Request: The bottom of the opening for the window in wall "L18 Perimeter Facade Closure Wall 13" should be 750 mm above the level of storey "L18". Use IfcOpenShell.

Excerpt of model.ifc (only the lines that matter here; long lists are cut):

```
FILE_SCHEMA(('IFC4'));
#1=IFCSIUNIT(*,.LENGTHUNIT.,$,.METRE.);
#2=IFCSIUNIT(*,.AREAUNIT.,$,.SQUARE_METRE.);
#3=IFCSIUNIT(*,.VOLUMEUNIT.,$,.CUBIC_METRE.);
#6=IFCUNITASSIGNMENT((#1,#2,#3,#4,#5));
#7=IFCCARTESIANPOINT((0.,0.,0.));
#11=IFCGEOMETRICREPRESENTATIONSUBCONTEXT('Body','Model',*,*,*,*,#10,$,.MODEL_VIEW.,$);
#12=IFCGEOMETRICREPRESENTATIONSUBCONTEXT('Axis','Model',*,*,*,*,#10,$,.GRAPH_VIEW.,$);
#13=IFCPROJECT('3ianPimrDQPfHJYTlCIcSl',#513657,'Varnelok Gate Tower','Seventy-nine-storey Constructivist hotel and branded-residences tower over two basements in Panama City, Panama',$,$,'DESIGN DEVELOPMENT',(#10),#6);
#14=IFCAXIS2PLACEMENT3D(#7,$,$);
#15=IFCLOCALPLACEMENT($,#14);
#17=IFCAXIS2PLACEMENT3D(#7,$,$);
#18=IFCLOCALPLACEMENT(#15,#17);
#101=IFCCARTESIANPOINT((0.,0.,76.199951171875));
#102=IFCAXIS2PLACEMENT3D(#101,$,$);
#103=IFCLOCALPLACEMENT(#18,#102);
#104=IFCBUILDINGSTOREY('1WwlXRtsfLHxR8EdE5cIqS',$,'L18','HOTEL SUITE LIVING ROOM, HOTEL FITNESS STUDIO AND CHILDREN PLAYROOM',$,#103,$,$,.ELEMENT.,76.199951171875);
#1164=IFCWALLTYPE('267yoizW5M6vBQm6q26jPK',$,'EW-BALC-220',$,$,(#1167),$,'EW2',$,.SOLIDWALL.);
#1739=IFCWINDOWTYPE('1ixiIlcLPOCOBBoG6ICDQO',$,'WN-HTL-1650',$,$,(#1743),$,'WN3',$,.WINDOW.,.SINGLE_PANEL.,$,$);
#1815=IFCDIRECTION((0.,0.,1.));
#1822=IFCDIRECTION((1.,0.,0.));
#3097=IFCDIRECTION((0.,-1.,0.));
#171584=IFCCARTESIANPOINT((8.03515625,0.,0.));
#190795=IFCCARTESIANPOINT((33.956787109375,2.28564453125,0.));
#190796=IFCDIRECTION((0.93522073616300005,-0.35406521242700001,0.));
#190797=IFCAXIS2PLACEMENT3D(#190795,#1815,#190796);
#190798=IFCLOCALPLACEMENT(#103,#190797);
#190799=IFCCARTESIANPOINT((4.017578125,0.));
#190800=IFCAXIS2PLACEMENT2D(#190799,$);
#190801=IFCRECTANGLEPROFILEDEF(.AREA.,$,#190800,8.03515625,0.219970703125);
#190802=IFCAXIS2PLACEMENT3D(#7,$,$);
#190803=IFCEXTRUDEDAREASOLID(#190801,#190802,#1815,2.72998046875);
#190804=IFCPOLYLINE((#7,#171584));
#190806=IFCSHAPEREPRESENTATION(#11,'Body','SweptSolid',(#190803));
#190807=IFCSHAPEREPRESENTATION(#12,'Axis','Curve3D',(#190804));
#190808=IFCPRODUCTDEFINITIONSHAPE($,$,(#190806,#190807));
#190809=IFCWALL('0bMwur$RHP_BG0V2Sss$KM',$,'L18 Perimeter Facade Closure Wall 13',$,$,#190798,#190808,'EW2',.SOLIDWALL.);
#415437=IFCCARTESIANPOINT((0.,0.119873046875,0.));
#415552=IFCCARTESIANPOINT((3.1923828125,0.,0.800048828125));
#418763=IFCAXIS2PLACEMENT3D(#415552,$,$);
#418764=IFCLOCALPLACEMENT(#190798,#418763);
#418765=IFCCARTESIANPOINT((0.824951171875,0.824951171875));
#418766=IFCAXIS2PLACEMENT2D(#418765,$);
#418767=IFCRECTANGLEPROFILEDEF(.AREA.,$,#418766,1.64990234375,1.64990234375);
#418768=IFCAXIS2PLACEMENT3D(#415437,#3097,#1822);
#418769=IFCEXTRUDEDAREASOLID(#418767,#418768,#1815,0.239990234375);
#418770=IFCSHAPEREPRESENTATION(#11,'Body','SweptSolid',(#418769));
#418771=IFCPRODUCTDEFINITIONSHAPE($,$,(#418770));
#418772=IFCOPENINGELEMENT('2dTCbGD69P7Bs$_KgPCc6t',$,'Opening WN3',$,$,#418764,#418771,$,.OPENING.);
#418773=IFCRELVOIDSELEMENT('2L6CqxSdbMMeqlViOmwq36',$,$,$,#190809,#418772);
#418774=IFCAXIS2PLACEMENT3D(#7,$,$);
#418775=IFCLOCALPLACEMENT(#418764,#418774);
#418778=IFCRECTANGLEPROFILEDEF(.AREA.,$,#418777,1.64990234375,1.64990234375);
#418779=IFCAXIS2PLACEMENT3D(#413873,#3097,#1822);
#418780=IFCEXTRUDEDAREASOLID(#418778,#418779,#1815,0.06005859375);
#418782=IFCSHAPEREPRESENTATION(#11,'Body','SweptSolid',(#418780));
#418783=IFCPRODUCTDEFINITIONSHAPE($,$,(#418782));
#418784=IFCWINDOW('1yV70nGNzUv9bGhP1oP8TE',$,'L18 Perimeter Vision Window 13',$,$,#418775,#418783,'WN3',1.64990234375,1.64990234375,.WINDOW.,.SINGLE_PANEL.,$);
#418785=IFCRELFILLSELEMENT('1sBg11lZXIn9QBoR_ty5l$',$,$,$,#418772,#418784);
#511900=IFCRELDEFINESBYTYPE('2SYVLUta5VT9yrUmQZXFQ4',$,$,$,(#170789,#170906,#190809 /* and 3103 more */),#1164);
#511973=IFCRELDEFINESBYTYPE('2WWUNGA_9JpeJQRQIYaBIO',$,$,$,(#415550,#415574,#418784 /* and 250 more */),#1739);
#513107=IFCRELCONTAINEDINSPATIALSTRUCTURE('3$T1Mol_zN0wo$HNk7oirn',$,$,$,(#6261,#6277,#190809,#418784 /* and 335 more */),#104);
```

```python
import numpy as np
import ifcopenshell
import ifcopenshell.api.geometry
import ifcopenshell.geom
import ifcopenshell.util.element
import ifcopenshell.util.placement
import ifcopenshell.util.shape
import ifcopenshell.util.unit

model = ifcopenshell.open("model.ifc")
unit_scale = ifcopenshell.util.unit.calculate_unit_scale(model)

window = model.by_guid("1yV70nGNzUv9bGhP1oP8TE")
opening = window.FillsVoids[0].RelatingOpeningElement
storey = ifcopenshell.util.element.get_container(window, ifc_class="IfcBuildingStorey")
level = ifcopenshell.util.placement.get_local_placement(storey.ObjectPlacement)[2, 3]

# The opening's origin need not be at the sill, so measure its lowest point.
shape = ifcopenshell.geom.create_shape(ifcopenshell.geom.settings(), opening)
bottom = ifcopenshell.util.shape.get_shape_bottom_elevation(shape, shape.geometry) / unit_scale
dz = level + 0.75 - bottom

shift = np.array([0.0, 0.0, dz])
# The window is placed relative to its opening, so it follows when the opening moves.
matrix = ifcopenshell.util.placement.get_local_placement(opening.ObjectPlacement)
matrix[:3, 3] += shift
ifcopenshell.api.geometry.edit_object_placement(
    model, product=opening, matrix=matrix, is_si=False, should_transform_children=True
)

print(f"moved by {dz * unit_scale:+.3f} m")

model.write("model_updated.ifc")
```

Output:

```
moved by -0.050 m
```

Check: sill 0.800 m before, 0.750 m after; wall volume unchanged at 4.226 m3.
